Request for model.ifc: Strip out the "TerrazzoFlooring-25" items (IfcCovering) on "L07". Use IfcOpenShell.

First a look at what the model holds.

```python
import ifcopenshell
import ifcopenshell.util.element

model = ifcopenshell.open("model.ifc")
print(model.schema)
storey = next(s for s in model.by_type("IfcBuildingStorey") if s.Name == "L07")
coverings = [e for e in ifcopenshell.util.element.get_decomposition(storey) if e.is_a("IfcCovering")]
seen = {}
for e in coverings:
    element_type = ifcopenshell.util.element.get_type(e)
    name = element_type.Name if element_type not in (None, e) else None
    seen[name] = seen.get(name, 0) + 1
for name, count in sorted(seen.items(), key=str):
    print(count, "x", name)
```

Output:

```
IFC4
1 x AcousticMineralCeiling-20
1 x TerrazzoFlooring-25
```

```python
import ifcopenshell
import ifcopenshell.api.root
import ifcopenshell.util.element

model = ifcopenshell.open("model.ifc")

storey = next(s for s in model.by_type("IfcBuildingStorey") if s.Name == "L07")
coverings = [e for e in ifcopenshell.util.element.get_decomposition(storey) if e.is_a("IfcCovering")]
targets = [e for e in coverings if (t := ifcopenshell.util.element.get_type(e)) not in (None, e) and t.Name == "TerrazzoFlooring-25"]

for e in targets:
    ifcopenshell.api.root.remove_product(model, product=e)
print(len(targets), "removed")

model.write("model_edited.ifc")
```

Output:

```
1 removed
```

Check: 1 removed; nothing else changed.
